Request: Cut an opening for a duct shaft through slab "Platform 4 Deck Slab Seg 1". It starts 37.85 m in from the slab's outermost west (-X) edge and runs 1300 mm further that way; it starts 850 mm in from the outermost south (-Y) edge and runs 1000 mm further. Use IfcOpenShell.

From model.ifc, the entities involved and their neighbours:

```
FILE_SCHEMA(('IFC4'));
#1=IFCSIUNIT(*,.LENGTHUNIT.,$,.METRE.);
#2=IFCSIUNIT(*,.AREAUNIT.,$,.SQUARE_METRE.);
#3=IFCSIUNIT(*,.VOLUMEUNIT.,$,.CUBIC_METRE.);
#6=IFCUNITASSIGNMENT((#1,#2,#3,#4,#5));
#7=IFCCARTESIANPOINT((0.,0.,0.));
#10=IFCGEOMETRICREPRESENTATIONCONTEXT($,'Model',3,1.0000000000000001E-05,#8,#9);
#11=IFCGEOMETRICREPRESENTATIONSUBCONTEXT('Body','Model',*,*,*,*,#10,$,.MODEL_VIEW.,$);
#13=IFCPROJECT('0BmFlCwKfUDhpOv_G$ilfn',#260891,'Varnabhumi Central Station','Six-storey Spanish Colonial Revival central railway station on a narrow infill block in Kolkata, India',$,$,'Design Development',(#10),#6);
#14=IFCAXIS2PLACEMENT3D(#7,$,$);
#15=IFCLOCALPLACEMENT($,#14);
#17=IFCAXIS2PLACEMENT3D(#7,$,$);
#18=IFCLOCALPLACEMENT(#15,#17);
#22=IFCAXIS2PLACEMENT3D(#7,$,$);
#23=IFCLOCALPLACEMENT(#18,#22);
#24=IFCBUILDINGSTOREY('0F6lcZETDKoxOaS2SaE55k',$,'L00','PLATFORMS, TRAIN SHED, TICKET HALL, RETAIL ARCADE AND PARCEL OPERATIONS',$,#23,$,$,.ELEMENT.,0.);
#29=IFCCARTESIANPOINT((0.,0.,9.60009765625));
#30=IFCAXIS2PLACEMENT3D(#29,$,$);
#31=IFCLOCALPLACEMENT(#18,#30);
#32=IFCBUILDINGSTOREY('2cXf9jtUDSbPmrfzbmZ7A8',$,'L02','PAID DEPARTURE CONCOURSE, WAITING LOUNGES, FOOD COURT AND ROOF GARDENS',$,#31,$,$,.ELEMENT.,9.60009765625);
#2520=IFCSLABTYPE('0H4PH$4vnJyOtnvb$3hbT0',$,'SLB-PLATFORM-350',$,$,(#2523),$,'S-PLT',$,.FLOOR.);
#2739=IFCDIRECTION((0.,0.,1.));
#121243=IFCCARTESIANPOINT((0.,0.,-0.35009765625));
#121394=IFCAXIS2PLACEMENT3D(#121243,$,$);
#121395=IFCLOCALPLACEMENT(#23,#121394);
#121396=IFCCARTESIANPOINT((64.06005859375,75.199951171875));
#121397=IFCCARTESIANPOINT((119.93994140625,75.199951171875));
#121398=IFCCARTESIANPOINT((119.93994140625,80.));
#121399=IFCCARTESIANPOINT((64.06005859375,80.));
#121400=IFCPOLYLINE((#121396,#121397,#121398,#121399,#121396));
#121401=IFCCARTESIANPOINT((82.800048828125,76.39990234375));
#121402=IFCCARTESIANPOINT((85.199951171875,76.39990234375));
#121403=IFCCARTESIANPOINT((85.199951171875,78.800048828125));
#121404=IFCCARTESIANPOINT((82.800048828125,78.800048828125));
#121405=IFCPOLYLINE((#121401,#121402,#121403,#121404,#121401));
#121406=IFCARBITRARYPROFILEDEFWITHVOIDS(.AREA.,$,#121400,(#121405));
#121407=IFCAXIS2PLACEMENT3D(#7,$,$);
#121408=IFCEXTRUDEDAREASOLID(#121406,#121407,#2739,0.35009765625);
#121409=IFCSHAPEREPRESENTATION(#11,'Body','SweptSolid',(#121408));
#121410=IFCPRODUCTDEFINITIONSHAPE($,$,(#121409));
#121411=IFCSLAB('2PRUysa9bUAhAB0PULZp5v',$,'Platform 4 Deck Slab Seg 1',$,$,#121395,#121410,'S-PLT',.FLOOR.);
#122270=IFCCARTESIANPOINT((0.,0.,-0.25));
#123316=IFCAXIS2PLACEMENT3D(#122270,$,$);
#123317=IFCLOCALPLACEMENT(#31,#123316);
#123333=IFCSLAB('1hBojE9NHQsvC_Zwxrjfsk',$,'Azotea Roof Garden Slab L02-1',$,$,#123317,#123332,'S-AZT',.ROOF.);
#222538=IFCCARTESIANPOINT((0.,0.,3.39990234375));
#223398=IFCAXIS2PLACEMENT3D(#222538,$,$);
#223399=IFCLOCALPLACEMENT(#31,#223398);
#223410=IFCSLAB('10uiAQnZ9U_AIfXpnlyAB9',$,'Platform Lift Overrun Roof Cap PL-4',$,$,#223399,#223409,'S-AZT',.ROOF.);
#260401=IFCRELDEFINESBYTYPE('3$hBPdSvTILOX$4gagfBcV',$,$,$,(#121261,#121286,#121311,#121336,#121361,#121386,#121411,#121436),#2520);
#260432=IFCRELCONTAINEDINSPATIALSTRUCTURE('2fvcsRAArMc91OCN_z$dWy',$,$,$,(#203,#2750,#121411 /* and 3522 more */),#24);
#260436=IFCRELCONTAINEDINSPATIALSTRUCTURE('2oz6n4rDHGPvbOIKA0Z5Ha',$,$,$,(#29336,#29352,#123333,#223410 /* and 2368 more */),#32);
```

```python
import numpy as np
import ifcopenshell
import ifcopenshell.api.feature
import ifcopenshell.api.geometry
import ifcopenshell.api.root
import ifcopenshell.geom
import ifcopenshell.util.placement
import ifcopenshell.util.representation
import ifcopenshell.util.shape
import ifcopenshell.util.unit

model = ifcopenshell.open("model.ifc")
unit_scale = ifcopenshell.util.unit.calculate_unit_scale(model)
settings = ifcopenshell.geom.settings()


def volume(element):
    """Net volume in cubic metres, openings subtracted."""
    shape = ifcopenshell.geom.create_shape(settings, element)
    return ifcopenshell.util.shape.get_volume(shape.geometry)


slab = model.by_guid("2PRUysa9bUAhAB0PULZp5v")
before = volume(slab)

# Extent in the slab's own axes, in metres. The edges named are its -X and -Y sides.
slab_shape = ifcopenshell.geom.create_shape(settings, slab)
vertices = ifcopenshell.util.shape.get_vertices(slab_shape.geometry)
x_min, y_min, bottom = vertices.min(axis=0)
top = vertices[:, 2].max()

opening = ifcopenshell.api.root.create_entity(model, ifc_class="IfcOpeningElement", name="Duct shaft opening", predefined_type="OPENING")
context = ifcopenshell.util.representation.get_context(model, "Model", "Body", "MODEL_VIEW")
width, depth = 1.3, 1
outline = [(0.0, 0.0), (width, 0.0), (width, depth), (0.0, depth), (0.0, 0.0)]
# Overshoot both faces by 50 mm so the cut is clean.
shape = ifcopenshell.api.geometry.add_slab_representation(
    model, context=context, depth=top - bottom + 0.1, polyline=outline
)
ifcopenshell.api.geometry.assign_representation(model, product=opening, representation=shape)

matrix = ifcopenshell.util.placement.get_local_placement(slab.ObjectPlacement)
matrix[:, 3] = matrix @ np.append(np.array([x_min + 37.85, y_min + 0.85, bottom - 0.05]) / unit_scale, 1.0)
ifcopenshell.api.geometry.edit_object_placement(model, product=opening, matrix=matrix, is_si=False)
ifcopenshell.api.feature.add_feature(model, feature=opening, element=slab)

after = volume(slab)

print(f"slab volume {before:.3f} -> {after:.3f} m3")

model.write("model_edited.ifc")
```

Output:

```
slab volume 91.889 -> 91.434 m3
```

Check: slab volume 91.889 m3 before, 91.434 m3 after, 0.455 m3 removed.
